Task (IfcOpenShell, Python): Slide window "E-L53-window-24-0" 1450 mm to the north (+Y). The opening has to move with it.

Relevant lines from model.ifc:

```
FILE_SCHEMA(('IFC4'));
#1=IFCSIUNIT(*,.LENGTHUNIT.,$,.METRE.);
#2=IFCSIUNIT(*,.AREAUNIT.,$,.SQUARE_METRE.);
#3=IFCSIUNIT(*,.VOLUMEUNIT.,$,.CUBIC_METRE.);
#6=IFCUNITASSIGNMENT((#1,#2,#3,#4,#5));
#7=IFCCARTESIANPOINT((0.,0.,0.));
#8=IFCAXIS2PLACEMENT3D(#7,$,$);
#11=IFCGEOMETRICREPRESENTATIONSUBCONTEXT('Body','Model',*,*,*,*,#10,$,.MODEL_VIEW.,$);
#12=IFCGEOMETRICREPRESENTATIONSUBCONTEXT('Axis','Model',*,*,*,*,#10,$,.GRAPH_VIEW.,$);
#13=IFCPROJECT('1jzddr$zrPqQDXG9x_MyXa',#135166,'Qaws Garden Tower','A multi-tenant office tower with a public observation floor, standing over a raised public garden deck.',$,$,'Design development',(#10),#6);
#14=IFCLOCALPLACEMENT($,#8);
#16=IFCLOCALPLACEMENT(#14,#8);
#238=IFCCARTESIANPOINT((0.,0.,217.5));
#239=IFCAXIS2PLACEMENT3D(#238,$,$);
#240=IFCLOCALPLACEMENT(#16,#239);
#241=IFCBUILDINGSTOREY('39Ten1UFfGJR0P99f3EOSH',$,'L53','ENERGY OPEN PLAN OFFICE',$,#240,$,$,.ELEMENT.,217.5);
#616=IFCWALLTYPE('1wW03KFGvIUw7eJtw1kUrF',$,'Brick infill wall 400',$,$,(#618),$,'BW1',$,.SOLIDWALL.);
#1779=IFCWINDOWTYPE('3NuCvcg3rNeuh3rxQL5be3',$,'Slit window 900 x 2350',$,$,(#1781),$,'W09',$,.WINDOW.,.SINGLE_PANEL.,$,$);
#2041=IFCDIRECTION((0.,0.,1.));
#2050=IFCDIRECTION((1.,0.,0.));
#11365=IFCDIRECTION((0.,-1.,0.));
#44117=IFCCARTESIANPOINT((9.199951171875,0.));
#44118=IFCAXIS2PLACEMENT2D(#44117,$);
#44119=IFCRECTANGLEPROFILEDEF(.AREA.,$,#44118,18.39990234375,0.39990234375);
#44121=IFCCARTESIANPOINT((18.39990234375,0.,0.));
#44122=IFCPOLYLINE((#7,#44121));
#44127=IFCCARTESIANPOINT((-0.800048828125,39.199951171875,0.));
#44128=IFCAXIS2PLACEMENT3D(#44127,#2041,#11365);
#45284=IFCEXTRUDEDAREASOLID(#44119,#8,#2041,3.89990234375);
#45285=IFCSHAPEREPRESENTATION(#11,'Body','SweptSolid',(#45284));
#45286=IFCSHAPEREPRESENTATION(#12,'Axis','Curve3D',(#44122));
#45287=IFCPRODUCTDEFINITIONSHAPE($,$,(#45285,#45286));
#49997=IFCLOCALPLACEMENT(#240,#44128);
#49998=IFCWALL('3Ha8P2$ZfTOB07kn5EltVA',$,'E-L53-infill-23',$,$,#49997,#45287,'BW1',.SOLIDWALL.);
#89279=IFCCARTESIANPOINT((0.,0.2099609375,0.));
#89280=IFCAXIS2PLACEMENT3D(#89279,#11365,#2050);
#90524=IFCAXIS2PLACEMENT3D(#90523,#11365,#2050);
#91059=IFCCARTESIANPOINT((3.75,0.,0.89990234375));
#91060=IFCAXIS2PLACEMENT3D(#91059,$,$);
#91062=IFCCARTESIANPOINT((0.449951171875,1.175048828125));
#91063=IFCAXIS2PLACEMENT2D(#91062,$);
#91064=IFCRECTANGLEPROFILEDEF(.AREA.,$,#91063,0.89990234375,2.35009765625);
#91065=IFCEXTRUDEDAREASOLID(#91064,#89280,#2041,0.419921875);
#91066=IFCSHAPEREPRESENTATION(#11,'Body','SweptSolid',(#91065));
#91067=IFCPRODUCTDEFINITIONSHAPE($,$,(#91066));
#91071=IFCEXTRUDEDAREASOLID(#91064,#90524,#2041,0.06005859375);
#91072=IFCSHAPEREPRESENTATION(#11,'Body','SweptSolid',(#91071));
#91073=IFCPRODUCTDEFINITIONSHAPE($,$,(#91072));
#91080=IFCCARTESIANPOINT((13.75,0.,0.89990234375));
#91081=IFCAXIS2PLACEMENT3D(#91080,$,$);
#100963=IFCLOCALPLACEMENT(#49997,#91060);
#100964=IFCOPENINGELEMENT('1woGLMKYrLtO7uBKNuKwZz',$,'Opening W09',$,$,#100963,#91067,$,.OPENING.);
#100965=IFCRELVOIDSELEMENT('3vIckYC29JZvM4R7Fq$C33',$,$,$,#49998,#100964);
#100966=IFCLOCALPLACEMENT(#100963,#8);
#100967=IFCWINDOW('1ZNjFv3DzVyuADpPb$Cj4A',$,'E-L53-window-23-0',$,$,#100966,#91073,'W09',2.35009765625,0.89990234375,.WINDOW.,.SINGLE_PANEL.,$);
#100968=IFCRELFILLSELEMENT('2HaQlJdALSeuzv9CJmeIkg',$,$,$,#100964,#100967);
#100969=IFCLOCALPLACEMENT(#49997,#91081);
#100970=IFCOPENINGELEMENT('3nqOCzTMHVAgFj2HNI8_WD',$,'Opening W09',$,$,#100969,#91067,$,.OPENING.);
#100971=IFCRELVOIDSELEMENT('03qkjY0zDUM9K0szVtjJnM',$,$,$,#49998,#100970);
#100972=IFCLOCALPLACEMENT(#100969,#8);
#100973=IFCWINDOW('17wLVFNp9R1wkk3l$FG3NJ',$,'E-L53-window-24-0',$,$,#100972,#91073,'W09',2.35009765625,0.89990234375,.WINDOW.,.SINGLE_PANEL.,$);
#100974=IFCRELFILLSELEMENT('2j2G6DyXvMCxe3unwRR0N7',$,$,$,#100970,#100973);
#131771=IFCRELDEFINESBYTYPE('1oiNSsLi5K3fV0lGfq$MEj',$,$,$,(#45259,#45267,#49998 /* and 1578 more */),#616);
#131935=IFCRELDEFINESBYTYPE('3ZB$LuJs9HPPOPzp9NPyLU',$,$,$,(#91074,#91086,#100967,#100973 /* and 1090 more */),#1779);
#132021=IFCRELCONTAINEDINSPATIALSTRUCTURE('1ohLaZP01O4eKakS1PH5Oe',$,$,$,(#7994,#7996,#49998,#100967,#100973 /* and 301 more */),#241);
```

```python
import ifcopenshell
import ifcopenshell.api.geometry
import ifcopenshell.util.placement
import ifcopenshell.util.unit

model = ifcopenshell.open("model.ifc")
unit_scale = ifcopenshell.util.unit.calculate_unit_scale(model)

window = model.by_id(100973)
opening = window.FillsVoids[0].RelatingOpeningElement
wall = opening.VoidsElements[0].RelatingBuildingElement

wall_matrix = ifcopenshell.util.placement.get_local_placement(wall.ObjectPlacement)
shift = wall_matrix[:3, 0] * -1.45 / unit_scale
before = ifcopenshell.util.placement.get_local_placement(window.ObjectPlacement)[:3, 3].copy()

# The window is placed relative to its opening, so it follows when the opening moves.
matrix = ifcopenshell.util.placement.get_local_placement(opening.ObjectPlacement)
matrix[:3, 3] += shift
ifcopenshell.api.geometry.edit_object_placement(
    model, product=opening, matrix=matrix, is_si=False, should_transform_children=True
)

after = ifcopenshell.util.placement.get_local_placement(window.ObjectPlacement)[:3, 3]
print("window moved by", (after - before).round(3) + 0.0)

model.write("model_v2.ifc")
```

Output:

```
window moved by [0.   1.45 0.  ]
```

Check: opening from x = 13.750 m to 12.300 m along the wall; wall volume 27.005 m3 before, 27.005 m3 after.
